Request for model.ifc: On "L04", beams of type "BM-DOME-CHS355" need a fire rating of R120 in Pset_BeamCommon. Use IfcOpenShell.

First a look at what the model holds.

```python
import ifcopenshell
import ifcopenshell.util.element

model = ifcopenshell.open("model.ifc")
print(model.schema)
storey = next(s for s in model.by_type("IfcBuildingStorey") if s.Name == "L04")
beams = [e for e in ifcopenshell.util.element.get_decomposition(storey) if e.is_a("IfcBeam")]
seen = {}
for e in beams:
    element_type = ifcopenshell.util.element.get_type(e)
    key = (element_type.Name if element_type != e and element_type else None, ifcopenshell.util.element.get_pset(e, "Pset_BeamCommon", "FireRating"))
    seen[key] = seen.get(key, 0) + 1
for (name, value), count in sorted(seen.items(), key=str):
    print(count, "x", name, "|", value)
```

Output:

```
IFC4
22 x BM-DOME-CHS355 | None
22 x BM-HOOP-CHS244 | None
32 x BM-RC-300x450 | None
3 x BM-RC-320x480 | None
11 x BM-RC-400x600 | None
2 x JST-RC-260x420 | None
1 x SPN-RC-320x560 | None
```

```python
import ifcopenshell
import ifcopenshell.api.pset
import ifcopenshell.util.element

model = ifcopenshell.open("model.ifc")

storey = next(s for s in model.by_type("IfcBuildingStorey") if s.Name == "L04")
beams = [e for e in ifcopenshell.util.element.get_decomposition(storey) if e.is_a("IfcBeam")]

count = 0
for e in beams:
    element_type = ifcopenshell.util.element.get_type(e)
    if element_type in (None, e) or element_type.Name != "BM-DOME-CHS355":
        continue
    # add_pset returns the element's existing set when there is one.
    pset = ifcopenshell.api.pset.add_pset(model, product=e, name="Pset_BeamCommon")
    ifcopenshell.api.pset.edit_pset(model, pset=pset, properties={"FireRating": "R120"})
    count += 1

print(count, "beams updated")

model.write("model_rev.ifc")
```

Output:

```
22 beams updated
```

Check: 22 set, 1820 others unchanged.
